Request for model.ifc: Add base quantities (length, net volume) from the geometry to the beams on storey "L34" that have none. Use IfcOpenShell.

First a look at what the model holds.

```python
import ifcopenshell
import ifcopenshell.util.element
import ifcopenshell.util.unit

model = ifcopenshell.open("model.ifc")
print(model.schema)
for unit_type in ("LENGTHUNIT", "AREAUNIT", "VOLUMEUNIT"):
    print(unit_type, ifcopenshell.util.unit.calculate_unit_scale(model, unit_type))
storey = next(s for s in model.by_type("IfcBuildingStorey") if s.Name == "L34")
beams = [e for e in ifcopenshell.util.element.get_decomposition(storey) if e.is_a("IfcBeam")]
for e in sorted(beams, key=lambda e: e.id()):
    print(e.id(), e.is_a(), e.Name, list(ifcopenshell.util.element.get_psets(e, qtos_only=True)), sep=" | ")
```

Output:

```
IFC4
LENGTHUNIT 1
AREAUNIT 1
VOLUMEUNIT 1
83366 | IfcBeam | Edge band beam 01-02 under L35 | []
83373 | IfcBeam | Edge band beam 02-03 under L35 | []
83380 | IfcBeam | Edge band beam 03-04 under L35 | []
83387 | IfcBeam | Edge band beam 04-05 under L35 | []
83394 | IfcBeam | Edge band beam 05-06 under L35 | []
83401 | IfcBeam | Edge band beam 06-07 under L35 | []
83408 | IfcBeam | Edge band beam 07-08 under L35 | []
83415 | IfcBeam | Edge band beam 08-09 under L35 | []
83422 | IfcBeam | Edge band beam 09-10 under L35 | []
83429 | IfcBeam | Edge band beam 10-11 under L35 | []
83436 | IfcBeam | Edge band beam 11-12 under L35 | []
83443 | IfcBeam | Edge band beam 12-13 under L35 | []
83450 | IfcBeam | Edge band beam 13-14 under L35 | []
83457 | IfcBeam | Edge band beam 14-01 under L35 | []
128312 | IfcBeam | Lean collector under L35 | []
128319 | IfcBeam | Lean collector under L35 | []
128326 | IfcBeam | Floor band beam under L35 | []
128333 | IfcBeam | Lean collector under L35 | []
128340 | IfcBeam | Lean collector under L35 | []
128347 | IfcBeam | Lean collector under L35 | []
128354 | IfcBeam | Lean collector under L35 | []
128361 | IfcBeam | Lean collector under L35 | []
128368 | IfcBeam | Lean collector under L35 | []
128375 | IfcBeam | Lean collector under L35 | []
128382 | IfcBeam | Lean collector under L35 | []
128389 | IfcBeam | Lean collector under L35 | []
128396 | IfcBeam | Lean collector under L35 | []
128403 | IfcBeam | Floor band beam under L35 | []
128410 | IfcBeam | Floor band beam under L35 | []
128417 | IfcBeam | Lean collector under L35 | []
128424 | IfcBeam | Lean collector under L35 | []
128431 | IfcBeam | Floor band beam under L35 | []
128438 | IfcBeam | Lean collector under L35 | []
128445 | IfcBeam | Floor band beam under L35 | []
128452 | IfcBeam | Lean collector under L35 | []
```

```python
import ifcopenshell
import ifcopenshell.api.pset
import ifcopenshell.geom
import ifcopenshell.util.element
import ifcopenshell.util.shape
import ifcopenshell.util.unit

model = ifcopenshell.open("model.ifc")
unit_scale = ifcopenshell.util.unit.calculate_unit_scale(model)
volume_scale = ifcopenshell.util.unit.calculate_unit_scale(model, "VOLUMEUNIT")
settings = ifcopenshell.geom.settings()

storey = next(s for s in model.by_type("IfcBuildingStorey") if s.Name == "L34")
beams = [e for e in ifcopenshell.util.element.get_decomposition(storey) if e.is_a("IfcBeam")]

for e in sorted(beams, key=lambda e: e.id()):
    if ifcopenshell.util.element.get_psets(e, qtos_only=True, should_inherit=False):
        continue
    # Geometry comes back in metres, in the element's own axes.
    shape = ifcopenshell.geom.create_shape(settings, e)
    values = {
        "Length": ifcopenshell.util.shape.get_max_xyz(shape.geometry) / unit_scale,
        "NetVolume": ifcopenshell.util.shape.get_volume(shape.geometry) / volume_scale,
    }
    qto = ifcopenshell.api.pset.add_qto(model, product=e, name="Qto_BeamBaseQuantities")
    ifcopenshell.api.pset.edit_qto(model, qto=qto, properties=values)
    print(e.id(), {k: round(v, 3) for k, v in values.items()})

model.write("model-out.ifc")
```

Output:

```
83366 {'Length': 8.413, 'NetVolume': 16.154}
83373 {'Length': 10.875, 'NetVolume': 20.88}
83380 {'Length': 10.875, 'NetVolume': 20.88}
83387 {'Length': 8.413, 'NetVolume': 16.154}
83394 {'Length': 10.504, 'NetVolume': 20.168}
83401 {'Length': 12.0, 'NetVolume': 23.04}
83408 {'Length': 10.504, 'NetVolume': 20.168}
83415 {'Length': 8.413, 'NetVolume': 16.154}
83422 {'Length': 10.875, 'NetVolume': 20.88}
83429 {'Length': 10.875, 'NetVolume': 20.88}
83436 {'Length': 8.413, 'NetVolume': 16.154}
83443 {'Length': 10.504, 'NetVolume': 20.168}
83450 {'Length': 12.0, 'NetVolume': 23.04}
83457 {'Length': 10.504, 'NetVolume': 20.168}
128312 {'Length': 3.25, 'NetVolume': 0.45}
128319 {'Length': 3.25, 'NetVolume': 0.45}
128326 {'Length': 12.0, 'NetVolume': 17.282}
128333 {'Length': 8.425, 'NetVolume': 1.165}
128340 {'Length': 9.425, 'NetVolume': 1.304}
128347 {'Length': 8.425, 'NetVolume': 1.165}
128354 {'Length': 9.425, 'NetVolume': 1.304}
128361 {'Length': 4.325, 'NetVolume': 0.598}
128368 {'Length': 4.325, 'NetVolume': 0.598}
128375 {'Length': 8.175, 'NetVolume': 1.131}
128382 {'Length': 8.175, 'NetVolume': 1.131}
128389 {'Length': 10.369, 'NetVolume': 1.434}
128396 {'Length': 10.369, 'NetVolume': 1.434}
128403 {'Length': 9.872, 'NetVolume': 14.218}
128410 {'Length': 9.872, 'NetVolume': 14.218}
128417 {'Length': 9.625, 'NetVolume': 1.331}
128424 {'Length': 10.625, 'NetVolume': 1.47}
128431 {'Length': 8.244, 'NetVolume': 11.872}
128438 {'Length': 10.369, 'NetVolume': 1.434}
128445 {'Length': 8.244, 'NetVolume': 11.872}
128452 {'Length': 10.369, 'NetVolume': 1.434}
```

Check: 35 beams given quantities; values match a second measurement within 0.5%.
